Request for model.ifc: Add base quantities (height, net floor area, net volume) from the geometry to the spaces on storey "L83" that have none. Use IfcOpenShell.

First a look at what the model holds.

```python
import ifcopenshell
import ifcopenshell.util.element
import ifcopenshell.util.unit

model = ifcopenshell.open("model.ifc")
print(model.schema)
for unit_type in ("LENGTHUNIT", "AREAUNIT", "VOLUMEUNIT"):
    print(unit_type, ifcopenshell.util.unit.calculate_unit_scale(model, unit_type))
storey = next(s for s in model.by_type("IfcBuildingStorey") if s.Name == "L83")
spaces = [e for e in ifcopenshell.util.element.get_decomposition(storey) if e.is_a("IfcSpace")]
for e in sorted(spaces, key=lambda e: e.id()):
    print(e.id(), e.is_a(), e.Name, list(ifcopenshell.util.element.get_psets(e, qtos_only=True)), sep=" | ")
```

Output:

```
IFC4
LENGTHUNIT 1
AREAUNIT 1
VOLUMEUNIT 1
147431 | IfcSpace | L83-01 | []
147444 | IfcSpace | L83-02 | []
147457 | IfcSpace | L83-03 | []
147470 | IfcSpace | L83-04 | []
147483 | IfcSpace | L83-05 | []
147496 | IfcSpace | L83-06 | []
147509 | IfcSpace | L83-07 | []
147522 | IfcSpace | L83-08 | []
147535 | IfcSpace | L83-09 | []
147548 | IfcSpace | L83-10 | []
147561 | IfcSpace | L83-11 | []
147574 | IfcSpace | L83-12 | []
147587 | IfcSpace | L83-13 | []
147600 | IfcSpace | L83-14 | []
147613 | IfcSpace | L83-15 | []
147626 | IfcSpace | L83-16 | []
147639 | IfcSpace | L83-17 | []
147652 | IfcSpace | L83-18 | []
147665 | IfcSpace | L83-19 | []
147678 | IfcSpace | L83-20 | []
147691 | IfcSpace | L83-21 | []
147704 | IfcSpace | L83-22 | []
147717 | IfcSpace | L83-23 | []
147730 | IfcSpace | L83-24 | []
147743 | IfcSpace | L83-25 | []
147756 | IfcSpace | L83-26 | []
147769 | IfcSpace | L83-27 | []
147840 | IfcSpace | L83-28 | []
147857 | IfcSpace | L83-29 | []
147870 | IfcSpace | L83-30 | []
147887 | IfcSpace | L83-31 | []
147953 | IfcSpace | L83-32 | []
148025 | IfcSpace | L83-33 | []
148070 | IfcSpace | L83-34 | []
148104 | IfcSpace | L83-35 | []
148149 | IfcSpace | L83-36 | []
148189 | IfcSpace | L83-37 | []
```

```python
import ifcopenshell
import ifcopenshell.api.pset
import ifcopenshell.geom
import ifcopenshell.util.element
import ifcopenshell.util.shape
import ifcopenshell.util.unit

model = ifcopenshell.open("model.ifc")
unit_scale = ifcopenshell.util.unit.calculate_unit_scale(model)
area_scale = ifcopenshell.util.unit.calculate_unit_scale(model, "AREAUNIT")
volume_scale = ifcopenshell.util.unit.calculate_unit_scale(model, "VOLUMEUNIT")
settings = ifcopenshell.geom.settings()

storey = next(s for s in model.by_type("IfcBuildingStorey") if s.Name == "L83")
spaces = [e for e in ifcopenshell.util.element.get_decomposition(storey) if e.is_a("IfcSpace")]

for e in sorted(spaces, key=lambda e: e.id()):
    if ifcopenshell.util.element.get_psets(e, qtos_only=True, should_inherit=False):
        continue
    # Geometry comes back in metres, in the element's own axes.
    shape = ifcopenshell.geom.create_shape(settings, e)
    values = {
        "Height": ifcopenshell.util.shape.get_z(shape.geometry) / unit_scale,
        "NetFloorArea": ifcopenshell.util.shape.get_footprint_area(shape.geometry) / area_scale,
        "NetVolume": ifcopenshell.util.shape.get_volume(shape.geometry) / volume_scale,
    }
    qto = ifcopenshell.api.pset.add_qto(model, product=e, name="Qto_SpaceBaseQuantities")
    ifcopenshell.api.pset.edit_qto(model, qto=qto, properties=values)
    print(e.id(), {k: round(v, 3) for k, v in values.items()})

model.write("model_rev.ifc")
```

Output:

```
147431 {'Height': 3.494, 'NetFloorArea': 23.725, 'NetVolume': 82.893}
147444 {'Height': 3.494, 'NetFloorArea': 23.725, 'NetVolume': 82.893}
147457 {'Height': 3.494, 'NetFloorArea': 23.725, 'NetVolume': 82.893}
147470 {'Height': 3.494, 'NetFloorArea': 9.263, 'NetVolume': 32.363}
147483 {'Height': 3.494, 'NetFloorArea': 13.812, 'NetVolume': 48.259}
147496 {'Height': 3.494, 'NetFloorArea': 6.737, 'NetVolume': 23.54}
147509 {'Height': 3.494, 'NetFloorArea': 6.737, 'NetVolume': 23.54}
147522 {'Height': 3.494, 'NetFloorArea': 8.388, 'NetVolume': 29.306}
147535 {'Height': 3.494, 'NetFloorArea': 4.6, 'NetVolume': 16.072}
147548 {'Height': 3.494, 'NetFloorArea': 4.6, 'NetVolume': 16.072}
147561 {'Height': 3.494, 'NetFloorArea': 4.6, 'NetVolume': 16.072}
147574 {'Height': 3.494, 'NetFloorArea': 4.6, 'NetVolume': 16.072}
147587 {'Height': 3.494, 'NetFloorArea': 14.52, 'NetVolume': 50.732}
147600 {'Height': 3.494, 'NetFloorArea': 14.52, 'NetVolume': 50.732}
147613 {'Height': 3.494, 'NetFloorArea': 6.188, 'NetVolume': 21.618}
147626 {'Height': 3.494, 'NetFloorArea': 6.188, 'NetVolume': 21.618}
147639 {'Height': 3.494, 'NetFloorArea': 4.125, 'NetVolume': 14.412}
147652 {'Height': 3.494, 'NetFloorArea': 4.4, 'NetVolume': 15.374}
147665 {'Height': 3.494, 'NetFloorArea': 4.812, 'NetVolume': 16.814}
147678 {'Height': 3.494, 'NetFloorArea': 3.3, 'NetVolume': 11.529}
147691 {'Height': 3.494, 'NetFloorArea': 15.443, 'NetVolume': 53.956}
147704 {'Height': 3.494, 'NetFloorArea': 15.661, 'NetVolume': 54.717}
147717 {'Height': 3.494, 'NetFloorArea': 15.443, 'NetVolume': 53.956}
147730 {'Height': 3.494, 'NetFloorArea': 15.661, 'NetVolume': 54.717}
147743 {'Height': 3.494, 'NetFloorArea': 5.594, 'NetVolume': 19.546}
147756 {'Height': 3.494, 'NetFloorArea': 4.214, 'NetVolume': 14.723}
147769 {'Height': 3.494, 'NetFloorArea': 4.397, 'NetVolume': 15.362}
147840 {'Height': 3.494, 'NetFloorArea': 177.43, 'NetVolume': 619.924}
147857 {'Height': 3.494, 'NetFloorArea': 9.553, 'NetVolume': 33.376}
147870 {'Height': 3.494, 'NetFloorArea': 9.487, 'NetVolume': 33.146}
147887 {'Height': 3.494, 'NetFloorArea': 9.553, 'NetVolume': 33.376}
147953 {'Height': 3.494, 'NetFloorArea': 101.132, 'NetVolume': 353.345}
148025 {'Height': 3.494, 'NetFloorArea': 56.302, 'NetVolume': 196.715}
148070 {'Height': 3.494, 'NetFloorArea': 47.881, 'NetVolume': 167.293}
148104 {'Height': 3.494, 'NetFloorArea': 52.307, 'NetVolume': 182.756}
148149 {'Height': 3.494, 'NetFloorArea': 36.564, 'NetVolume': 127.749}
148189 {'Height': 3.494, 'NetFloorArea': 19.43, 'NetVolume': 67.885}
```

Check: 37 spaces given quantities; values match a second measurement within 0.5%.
